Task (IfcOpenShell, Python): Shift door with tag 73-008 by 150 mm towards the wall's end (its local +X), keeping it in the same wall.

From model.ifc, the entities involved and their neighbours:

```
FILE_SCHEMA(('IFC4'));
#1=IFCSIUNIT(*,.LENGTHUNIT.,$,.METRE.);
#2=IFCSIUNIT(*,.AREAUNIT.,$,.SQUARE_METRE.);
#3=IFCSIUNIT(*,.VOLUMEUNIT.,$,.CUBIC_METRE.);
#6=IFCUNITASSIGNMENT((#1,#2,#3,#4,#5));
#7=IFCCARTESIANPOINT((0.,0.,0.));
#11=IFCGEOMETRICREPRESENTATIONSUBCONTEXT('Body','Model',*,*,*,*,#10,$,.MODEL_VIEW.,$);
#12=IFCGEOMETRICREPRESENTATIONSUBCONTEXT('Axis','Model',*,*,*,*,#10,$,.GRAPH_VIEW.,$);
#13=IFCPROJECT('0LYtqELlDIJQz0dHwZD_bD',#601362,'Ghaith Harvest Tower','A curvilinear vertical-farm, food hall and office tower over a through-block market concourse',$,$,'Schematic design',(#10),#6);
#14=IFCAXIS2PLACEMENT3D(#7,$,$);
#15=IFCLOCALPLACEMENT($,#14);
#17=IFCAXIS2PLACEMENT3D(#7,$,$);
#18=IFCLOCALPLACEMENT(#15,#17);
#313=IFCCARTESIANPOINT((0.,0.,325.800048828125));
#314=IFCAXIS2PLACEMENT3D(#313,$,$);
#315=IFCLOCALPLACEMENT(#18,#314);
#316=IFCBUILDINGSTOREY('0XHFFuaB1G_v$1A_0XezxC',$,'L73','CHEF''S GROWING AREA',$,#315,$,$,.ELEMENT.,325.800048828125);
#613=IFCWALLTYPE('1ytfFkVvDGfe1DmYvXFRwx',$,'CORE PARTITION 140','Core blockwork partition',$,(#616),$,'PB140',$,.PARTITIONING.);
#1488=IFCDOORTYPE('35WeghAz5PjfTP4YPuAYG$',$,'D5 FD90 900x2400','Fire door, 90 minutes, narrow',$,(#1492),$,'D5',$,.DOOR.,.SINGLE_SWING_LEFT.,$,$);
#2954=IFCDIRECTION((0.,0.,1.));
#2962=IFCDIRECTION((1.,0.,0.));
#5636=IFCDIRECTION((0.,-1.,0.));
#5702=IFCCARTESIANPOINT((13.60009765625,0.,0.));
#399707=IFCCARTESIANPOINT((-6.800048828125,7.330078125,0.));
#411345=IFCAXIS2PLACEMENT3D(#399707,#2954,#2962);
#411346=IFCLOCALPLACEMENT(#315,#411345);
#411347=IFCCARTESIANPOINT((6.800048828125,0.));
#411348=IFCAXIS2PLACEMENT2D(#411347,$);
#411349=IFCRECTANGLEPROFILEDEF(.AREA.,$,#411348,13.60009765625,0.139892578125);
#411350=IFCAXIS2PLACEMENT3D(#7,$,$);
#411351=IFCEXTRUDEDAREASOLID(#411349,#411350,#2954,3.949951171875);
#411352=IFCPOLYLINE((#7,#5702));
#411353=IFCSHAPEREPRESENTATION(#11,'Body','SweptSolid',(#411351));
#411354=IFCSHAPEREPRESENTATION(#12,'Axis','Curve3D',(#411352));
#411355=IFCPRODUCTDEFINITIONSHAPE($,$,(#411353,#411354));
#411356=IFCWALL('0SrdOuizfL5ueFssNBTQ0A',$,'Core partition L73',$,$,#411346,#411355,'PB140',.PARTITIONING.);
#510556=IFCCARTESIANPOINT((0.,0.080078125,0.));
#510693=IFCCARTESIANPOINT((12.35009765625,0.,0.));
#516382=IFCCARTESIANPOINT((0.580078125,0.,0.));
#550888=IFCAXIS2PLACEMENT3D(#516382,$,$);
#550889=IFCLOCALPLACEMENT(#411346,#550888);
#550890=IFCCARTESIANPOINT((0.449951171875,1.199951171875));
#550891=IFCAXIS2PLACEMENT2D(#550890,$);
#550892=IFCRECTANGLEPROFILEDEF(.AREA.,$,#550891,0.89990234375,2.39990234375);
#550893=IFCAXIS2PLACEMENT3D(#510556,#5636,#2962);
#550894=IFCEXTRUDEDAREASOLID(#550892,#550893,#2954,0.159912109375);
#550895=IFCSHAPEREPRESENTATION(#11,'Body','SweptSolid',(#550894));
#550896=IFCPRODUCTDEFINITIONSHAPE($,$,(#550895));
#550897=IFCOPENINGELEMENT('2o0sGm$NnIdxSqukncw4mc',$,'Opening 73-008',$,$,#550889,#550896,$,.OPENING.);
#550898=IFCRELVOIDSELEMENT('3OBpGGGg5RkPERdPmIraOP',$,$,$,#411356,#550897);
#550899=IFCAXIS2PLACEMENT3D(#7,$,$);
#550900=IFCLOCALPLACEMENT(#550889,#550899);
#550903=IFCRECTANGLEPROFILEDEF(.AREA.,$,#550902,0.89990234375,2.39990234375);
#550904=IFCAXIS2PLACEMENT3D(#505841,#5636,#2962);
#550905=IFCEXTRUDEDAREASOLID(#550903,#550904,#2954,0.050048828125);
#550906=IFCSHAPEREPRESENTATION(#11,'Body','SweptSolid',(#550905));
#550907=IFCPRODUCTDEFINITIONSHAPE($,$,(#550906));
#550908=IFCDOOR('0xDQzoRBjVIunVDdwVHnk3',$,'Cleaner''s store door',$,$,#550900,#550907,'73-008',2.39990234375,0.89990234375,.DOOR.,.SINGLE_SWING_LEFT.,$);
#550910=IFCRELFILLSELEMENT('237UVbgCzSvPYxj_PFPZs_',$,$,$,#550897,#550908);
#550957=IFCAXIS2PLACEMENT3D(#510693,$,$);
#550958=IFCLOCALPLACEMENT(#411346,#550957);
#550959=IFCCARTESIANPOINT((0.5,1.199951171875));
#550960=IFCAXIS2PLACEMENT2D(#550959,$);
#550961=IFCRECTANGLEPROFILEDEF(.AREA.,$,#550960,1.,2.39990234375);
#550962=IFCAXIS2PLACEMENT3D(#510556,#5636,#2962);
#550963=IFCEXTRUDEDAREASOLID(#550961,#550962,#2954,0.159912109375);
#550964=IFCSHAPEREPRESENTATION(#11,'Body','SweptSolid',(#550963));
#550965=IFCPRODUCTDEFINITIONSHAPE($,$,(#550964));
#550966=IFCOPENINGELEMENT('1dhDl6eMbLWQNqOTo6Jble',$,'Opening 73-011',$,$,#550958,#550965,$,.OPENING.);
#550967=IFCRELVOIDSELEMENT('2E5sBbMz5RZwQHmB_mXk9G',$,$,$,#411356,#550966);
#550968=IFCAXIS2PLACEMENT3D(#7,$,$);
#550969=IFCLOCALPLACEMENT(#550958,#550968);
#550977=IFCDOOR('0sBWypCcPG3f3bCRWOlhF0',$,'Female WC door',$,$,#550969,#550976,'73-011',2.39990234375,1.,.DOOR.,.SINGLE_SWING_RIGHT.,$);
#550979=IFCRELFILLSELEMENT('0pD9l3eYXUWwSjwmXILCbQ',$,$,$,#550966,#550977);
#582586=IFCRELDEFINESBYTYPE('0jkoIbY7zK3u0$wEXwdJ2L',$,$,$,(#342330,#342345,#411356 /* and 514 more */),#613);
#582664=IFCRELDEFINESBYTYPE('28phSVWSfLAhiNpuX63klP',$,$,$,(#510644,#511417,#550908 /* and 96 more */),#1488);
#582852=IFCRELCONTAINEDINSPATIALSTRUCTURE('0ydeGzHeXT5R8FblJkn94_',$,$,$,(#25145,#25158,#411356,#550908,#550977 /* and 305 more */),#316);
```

```python
import ifcopenshell
import ifcopenshell.api.geometry
import ifcopenshell.util.placement

model = ifcopenshell.open("model.ifc")

door = model.by_guid("0xDQzoRBjVIunVDdwVHnk3")
opening = door.FillsVoids[0].RelatingOpeningElement
wall = opening.VoidsElements[0].RelatingBuildingElement

wall_matrix = ifcopenshell.util.placement.get_local_placement(wall.ObjectPlacement)
shift = wall_matrix[:3, 0] * 0.15
before = ifcopenshell.util.placement.get_local_placement(door.ObjectPlacement)[:3, 3].copy()

# The door is placed relative to its opening, so it follows when the opening moves.
matrix = ifcopenshell.util.placement.get_local_placement(opening.ObjectPlacement)
matrix[:3, 3] += shift
ifcopenshell.api.geometry.edit_object_placement(
    model, product=opening, matrix=matrix, is_si=False, should_transform_children=True
)

after = ifcopenshell.util.placement.get_local_placement(door.ObjectPlacement)[:3, 3]
print("door moved by", (after - before).round(3) + 0.0)

model.write("model-out.ifc")
```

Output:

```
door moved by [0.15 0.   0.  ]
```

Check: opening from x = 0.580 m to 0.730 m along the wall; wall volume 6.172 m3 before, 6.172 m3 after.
